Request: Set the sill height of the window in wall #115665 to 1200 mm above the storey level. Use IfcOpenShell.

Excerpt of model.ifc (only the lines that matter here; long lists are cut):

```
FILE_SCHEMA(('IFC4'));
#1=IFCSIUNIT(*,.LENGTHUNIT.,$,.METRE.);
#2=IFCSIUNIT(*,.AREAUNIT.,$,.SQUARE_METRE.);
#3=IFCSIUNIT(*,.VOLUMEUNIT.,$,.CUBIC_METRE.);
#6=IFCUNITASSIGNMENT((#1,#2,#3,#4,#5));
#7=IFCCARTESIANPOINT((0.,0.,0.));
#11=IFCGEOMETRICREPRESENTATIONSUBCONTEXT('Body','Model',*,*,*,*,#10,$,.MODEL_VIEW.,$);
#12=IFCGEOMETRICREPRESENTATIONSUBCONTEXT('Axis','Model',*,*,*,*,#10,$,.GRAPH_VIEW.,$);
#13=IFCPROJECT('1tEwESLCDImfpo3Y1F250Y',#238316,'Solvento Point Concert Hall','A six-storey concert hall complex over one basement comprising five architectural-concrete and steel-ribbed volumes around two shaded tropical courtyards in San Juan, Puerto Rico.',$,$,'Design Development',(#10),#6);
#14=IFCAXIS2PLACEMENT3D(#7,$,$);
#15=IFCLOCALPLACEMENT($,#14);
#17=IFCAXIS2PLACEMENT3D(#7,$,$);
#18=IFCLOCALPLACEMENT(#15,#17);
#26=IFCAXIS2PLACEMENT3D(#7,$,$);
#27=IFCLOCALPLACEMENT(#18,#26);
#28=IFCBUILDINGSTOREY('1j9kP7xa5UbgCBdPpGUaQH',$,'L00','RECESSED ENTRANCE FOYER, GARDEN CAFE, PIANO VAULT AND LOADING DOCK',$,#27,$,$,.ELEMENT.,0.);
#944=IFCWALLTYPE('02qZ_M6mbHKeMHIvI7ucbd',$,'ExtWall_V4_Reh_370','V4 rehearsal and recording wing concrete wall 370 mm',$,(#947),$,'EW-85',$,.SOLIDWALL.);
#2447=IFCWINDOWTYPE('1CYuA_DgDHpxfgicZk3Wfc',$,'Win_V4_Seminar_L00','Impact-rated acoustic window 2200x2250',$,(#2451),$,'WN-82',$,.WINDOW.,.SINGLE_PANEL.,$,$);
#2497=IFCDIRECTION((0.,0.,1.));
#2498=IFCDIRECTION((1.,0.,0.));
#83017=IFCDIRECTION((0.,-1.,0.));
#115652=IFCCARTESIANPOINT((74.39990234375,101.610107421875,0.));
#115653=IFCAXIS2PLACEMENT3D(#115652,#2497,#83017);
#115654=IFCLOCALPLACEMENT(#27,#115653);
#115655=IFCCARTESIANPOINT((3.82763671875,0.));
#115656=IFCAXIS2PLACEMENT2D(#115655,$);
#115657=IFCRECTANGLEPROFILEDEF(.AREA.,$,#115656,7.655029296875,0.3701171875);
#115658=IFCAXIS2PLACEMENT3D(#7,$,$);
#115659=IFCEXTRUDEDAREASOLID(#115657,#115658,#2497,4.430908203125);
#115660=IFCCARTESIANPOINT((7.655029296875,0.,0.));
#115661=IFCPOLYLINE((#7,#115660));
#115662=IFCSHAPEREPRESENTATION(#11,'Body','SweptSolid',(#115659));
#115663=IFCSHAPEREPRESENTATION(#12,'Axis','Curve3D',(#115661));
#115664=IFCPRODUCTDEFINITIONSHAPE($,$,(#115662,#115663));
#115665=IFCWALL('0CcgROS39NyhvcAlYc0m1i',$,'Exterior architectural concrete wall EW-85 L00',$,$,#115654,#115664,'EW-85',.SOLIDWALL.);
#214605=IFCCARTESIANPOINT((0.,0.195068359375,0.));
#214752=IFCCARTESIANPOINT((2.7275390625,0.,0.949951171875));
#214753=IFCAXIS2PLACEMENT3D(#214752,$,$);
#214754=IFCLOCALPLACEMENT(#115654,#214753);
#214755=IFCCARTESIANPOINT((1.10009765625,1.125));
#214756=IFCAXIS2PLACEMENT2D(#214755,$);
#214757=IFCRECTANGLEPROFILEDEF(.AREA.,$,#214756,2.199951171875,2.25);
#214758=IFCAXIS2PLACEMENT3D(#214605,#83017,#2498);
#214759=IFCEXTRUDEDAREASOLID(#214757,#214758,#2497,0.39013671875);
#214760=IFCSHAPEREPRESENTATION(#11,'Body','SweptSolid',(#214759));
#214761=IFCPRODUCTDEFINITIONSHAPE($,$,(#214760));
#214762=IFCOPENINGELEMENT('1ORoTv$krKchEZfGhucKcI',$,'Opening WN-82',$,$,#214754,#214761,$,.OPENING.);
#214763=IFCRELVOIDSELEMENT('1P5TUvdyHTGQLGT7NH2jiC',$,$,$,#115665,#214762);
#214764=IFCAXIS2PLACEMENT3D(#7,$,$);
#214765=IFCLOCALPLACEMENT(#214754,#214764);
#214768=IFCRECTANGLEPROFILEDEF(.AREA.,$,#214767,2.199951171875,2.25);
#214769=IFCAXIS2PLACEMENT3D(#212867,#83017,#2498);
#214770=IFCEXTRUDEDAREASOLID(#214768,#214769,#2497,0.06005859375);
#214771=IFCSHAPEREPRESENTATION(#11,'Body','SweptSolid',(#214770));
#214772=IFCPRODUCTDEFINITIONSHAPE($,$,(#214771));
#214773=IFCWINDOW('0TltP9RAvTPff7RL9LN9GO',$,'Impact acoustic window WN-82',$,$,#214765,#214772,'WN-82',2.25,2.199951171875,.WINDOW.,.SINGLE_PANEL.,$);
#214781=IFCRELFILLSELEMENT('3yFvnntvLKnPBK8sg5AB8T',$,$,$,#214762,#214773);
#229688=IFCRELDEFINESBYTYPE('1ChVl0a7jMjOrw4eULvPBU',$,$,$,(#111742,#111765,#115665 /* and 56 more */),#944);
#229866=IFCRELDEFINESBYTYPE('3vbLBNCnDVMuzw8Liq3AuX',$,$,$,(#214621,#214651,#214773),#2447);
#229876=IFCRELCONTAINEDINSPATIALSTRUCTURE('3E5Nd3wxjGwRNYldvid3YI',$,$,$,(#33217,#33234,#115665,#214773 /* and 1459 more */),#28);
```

```python
import numpy as np
import ifcopenshell
import ifcopenshell.api.geometry
import ifcopenshell.geom
import ifcopenshell.util.element
import ifcopenshell.util.placement
import ifcopenshell.util.shape
import ifcopenshell.util.unit

model = ifcopenshell.open("model.ifc")
unit_scale = ifcopenshell.util.unit.calculate_unit_scale(model)

window = model.by_guid("0TltP9RAvTPff7RL9LN9GO")
opening = window.FillsVoids[0].RelatingOpeningElement
storey = ifcopenshell.util.element.get_container(window, ifc_class="IfcBuildingStorey")
level = ifcopenshell.util.placement.get_local_placement(storey.ObjectPlacement)[2, 3]

# The opening's origin need not be at the sill, so measure its lowest point.
shape = ifcopenshell.geom.create_shape(ifcopenshell.geom.settings(), opening)
bottom = ifcopenshell.util.shape.get_shape_bottom_elevation(shape, shape.geometry) / unit_scale
dz = level + 1.2 / unit_scale - bottom

shift = np.array([0.0, 0.0, dz])
# The window is placed relative to its opening, so it follows when the opening moves.
matrix = ifcopenshell.util.placement.get_local_placement(opening.ObjectPlacement)
matrix[:3, 3] += shift
ifcopenshell.api.geometry.edit_object_placement(
    model, product=opening, matrix=matrix, is_si=False, should_transform_children=True
)

print(f"moved by {dz * unit_scale:+.3f} m")

model.write("model_rev.ifc")
```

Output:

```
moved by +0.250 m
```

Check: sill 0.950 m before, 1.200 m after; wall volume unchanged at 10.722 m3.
